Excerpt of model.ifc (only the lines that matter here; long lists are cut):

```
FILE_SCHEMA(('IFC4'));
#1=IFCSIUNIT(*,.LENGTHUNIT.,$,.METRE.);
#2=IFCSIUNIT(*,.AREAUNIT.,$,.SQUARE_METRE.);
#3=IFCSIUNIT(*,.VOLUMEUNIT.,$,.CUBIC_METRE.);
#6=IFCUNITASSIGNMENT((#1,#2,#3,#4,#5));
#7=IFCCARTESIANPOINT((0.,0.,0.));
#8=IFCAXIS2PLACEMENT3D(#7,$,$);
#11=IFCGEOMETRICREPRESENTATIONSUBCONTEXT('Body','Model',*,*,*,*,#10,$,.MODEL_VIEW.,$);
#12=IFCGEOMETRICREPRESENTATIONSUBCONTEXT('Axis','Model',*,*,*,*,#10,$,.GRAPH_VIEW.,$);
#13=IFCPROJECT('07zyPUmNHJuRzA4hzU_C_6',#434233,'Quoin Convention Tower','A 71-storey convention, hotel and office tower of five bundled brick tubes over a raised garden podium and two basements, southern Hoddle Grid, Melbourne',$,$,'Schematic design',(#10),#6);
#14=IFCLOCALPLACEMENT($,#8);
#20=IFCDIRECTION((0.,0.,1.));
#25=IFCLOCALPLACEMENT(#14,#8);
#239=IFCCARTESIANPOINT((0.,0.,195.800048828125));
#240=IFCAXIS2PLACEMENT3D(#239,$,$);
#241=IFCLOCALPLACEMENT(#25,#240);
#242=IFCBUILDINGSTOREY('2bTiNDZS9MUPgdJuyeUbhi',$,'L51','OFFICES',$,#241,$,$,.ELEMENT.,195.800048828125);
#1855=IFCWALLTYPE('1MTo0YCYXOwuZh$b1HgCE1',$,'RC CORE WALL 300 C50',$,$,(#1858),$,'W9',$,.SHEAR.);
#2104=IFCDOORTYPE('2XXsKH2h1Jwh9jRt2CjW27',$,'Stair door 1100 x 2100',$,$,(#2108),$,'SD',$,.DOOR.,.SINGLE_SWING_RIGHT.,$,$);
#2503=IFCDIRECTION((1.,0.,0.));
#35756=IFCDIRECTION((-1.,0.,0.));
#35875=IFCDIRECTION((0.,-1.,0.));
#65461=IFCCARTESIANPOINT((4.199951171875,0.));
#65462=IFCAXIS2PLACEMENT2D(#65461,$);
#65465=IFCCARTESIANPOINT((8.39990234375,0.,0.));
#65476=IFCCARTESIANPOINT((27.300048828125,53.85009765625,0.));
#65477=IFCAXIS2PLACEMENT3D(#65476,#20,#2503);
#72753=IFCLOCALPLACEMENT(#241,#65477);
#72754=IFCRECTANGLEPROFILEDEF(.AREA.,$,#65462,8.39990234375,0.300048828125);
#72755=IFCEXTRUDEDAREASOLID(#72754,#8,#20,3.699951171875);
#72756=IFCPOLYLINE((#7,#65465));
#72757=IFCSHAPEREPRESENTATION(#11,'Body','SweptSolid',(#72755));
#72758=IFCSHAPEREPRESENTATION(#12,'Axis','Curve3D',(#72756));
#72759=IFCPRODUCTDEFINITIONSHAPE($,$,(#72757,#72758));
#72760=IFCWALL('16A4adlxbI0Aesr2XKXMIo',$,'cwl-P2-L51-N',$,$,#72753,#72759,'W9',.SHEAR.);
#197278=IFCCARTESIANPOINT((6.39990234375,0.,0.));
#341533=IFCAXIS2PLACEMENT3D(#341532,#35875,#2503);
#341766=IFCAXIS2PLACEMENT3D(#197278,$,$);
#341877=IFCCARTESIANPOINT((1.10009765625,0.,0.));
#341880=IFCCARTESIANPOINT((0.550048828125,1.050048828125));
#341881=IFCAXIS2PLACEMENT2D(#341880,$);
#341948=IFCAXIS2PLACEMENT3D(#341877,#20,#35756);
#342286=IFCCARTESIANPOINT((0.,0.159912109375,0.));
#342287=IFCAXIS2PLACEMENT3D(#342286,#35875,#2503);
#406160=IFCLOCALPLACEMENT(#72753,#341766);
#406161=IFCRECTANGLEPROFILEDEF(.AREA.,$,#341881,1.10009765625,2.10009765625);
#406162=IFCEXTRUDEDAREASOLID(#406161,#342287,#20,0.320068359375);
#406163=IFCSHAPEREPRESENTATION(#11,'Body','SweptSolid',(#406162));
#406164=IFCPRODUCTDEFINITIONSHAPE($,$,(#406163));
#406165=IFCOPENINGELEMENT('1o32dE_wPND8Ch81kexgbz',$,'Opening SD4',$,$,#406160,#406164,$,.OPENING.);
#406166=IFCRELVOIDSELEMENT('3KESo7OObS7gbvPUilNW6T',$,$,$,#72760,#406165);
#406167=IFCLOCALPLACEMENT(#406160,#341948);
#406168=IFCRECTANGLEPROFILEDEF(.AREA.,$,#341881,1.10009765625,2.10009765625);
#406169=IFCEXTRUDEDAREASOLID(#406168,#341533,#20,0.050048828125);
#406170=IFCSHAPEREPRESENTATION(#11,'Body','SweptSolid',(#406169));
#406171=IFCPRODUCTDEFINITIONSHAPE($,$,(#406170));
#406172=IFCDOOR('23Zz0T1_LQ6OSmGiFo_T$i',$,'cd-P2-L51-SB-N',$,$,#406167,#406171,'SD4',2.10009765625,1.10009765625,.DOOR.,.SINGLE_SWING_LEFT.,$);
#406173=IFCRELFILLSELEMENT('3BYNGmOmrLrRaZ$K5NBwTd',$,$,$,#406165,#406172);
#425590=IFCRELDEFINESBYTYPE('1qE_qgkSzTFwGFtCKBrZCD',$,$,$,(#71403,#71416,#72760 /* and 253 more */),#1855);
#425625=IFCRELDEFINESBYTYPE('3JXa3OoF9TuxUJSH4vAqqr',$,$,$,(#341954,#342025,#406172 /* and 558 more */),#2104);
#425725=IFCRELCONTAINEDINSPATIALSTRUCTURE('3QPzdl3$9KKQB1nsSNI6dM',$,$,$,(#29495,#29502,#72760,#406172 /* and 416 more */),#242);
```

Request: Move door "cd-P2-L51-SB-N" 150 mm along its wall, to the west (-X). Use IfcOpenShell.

```python
import ifcopenshell
import ifcopenshell.api.geometry
import ifcopenshell.util.placement

model = ifcopenshell.open("model.ifc")

door = model.by_guid("23Zz0T1_LQ6OSmGiFo_T$i")
opening = door.FillsVoids[0].RelatingOpeningElement
wall = opening.VoidsElements[0].RelatingBuildingElement

wall_matrix = ifcopenshell.util.placement.get_local_placement(wall.ObjectPlacement)
shift = wall_matrix[:3, 0] * -0.15
before = ifcopenshell.util.placement.get_local_placement(door.ObjectPlacement)[:3, 3].copy()

# The door is placed relative to its opening, so it follows when the opening moves.
matrix = ifcopenshell.util.placement.get_local_placement(opening.ObjectPlacement)
matrix[:3, 3] += shift
ifcopenshell.api.geometry.edit_object_placement(
    model, product=opening, matrix=matrix, is_si=False, should_transform_children=True
)

after = ifcopenshell.util.placement.get_local_placement(door.ObjectPlacement)[:3, 3]
print("door moved by", (after - before).round(3) + 0.0)

model.write("model-out.ifc")
```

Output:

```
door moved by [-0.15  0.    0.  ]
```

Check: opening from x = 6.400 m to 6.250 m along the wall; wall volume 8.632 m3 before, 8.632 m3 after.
